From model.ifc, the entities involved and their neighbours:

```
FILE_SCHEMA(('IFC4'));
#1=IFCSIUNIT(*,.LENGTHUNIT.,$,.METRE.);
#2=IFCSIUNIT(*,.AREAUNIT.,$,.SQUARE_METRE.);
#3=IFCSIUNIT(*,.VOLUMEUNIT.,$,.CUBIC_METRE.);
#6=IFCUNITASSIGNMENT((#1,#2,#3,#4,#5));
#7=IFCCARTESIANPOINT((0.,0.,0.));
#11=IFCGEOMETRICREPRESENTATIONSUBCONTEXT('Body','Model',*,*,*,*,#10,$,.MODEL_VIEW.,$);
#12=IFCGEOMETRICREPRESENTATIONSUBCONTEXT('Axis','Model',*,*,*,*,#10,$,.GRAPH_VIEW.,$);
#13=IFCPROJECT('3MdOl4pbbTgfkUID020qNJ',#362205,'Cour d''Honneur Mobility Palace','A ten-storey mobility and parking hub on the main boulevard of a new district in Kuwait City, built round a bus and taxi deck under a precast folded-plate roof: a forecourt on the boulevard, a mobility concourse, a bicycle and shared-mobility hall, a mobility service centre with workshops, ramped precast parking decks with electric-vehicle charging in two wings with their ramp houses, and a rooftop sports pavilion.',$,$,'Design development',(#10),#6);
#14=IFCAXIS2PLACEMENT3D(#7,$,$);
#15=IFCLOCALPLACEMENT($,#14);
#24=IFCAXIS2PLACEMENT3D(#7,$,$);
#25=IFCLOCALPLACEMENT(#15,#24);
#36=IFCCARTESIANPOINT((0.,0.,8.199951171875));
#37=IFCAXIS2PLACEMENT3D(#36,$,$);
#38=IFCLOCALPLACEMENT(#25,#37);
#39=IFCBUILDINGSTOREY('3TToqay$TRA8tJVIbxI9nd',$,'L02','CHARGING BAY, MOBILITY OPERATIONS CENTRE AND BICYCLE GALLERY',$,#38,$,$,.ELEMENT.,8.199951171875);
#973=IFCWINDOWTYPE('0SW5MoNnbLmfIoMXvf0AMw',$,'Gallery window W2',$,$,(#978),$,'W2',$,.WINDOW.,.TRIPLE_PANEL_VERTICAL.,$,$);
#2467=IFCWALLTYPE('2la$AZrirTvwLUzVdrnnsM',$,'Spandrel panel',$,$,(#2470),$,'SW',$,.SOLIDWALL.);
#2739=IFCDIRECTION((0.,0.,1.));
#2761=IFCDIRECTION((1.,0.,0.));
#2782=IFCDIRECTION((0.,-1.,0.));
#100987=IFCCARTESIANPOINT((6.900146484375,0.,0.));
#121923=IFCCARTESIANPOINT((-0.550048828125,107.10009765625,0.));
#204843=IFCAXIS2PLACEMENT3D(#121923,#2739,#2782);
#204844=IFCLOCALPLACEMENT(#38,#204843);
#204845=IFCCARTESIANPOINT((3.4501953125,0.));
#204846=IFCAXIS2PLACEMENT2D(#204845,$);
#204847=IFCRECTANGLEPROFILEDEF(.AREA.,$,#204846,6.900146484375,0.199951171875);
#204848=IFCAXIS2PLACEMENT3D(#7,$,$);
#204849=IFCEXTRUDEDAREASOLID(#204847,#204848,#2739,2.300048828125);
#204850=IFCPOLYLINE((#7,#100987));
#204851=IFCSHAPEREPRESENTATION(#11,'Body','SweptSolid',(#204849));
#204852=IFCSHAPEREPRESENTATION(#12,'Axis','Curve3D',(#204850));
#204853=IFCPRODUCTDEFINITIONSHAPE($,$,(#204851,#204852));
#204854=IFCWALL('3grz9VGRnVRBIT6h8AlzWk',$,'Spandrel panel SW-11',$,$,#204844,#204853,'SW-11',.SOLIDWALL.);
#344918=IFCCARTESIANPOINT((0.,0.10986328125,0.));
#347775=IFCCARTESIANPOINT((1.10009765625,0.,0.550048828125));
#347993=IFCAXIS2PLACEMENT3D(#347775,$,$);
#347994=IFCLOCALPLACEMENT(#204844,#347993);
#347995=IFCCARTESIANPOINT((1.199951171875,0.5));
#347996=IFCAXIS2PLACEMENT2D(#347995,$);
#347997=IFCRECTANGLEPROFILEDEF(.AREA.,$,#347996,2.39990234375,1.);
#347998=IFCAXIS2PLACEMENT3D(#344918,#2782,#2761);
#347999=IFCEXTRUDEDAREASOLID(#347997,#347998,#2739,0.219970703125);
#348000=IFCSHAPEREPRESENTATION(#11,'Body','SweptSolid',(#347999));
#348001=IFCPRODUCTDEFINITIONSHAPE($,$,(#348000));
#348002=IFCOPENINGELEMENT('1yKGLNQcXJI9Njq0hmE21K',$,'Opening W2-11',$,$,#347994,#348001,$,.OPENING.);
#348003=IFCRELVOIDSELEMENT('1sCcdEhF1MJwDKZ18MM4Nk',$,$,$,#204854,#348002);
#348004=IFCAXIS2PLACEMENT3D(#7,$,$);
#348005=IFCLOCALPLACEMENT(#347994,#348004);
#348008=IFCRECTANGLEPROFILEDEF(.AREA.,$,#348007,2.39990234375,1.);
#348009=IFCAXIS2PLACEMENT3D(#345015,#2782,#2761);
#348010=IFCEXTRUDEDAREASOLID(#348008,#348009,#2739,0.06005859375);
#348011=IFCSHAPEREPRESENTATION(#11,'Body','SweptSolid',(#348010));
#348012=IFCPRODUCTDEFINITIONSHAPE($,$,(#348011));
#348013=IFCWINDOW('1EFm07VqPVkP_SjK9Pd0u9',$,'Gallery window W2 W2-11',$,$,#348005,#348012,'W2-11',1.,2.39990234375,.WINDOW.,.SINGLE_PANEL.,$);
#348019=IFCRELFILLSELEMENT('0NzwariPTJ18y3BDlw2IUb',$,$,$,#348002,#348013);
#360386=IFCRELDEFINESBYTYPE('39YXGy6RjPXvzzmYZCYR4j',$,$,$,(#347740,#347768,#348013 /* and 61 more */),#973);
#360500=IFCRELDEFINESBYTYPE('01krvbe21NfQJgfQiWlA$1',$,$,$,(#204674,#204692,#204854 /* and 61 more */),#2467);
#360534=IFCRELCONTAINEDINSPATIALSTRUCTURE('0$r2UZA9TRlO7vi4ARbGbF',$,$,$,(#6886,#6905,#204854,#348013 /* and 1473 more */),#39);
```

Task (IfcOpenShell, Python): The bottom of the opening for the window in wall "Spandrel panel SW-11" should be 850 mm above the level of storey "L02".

```python
import numpy as np
import ifcopenshell
import ifcopenshell.api.geometry
import ifcopenshell.geom
import ifcopenshell.util.element
import ifcopenshell.util.placement
import ifcopenshell.util.shape
import ifcopenshell.util.unit

model = ifcopenshell.open("model.ifc")
unit_scale = ifcopenshell.util.unit.calculate_unit_scale(model)

window = model.by_guid("1EFm07VqPVkP_SjK9Pd0u9")
opening = window.FillsVoids[0].RelatingOpeningElement
storey = ifcopenshell.util.element.get_container(window, ifc_class="IfcBuildingStorey")
level = ifcopenshell.util.placement.get_local_placement(storey.ObjectPlacement)[2, 3]

# The opening's origin need not be at the sill, so measure its lowest point.
shape = ifcopenshell.geom.create_shape(ifcopenshell.geom.settings(), opening)
bottom = ifcopenshell.util.shape.get_shape_bottom_elevation(shape, shape.geometry) / unit_scale
dz = level + 0.85 / unit_scale - bottom

shift = np.array([0.0, 0.0, dz])
# The window is placed relative to its opening, so it follows when the opening moves.
matrix = ifcopenshell.util.placement.get_local_placement(opening.ObjectPlacement)
matrix[:3, 3] += shift
ifcopenshell.api.geometry.edit_object_placement(
    model, product=opening, matrix=matrix, is_si=False, should_transform_children=True
)

print(f"moved by {dz * unit_scale:+.3f} m")

model.write("model_rev.ifc")
```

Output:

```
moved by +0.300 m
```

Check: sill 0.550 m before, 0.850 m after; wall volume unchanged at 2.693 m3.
